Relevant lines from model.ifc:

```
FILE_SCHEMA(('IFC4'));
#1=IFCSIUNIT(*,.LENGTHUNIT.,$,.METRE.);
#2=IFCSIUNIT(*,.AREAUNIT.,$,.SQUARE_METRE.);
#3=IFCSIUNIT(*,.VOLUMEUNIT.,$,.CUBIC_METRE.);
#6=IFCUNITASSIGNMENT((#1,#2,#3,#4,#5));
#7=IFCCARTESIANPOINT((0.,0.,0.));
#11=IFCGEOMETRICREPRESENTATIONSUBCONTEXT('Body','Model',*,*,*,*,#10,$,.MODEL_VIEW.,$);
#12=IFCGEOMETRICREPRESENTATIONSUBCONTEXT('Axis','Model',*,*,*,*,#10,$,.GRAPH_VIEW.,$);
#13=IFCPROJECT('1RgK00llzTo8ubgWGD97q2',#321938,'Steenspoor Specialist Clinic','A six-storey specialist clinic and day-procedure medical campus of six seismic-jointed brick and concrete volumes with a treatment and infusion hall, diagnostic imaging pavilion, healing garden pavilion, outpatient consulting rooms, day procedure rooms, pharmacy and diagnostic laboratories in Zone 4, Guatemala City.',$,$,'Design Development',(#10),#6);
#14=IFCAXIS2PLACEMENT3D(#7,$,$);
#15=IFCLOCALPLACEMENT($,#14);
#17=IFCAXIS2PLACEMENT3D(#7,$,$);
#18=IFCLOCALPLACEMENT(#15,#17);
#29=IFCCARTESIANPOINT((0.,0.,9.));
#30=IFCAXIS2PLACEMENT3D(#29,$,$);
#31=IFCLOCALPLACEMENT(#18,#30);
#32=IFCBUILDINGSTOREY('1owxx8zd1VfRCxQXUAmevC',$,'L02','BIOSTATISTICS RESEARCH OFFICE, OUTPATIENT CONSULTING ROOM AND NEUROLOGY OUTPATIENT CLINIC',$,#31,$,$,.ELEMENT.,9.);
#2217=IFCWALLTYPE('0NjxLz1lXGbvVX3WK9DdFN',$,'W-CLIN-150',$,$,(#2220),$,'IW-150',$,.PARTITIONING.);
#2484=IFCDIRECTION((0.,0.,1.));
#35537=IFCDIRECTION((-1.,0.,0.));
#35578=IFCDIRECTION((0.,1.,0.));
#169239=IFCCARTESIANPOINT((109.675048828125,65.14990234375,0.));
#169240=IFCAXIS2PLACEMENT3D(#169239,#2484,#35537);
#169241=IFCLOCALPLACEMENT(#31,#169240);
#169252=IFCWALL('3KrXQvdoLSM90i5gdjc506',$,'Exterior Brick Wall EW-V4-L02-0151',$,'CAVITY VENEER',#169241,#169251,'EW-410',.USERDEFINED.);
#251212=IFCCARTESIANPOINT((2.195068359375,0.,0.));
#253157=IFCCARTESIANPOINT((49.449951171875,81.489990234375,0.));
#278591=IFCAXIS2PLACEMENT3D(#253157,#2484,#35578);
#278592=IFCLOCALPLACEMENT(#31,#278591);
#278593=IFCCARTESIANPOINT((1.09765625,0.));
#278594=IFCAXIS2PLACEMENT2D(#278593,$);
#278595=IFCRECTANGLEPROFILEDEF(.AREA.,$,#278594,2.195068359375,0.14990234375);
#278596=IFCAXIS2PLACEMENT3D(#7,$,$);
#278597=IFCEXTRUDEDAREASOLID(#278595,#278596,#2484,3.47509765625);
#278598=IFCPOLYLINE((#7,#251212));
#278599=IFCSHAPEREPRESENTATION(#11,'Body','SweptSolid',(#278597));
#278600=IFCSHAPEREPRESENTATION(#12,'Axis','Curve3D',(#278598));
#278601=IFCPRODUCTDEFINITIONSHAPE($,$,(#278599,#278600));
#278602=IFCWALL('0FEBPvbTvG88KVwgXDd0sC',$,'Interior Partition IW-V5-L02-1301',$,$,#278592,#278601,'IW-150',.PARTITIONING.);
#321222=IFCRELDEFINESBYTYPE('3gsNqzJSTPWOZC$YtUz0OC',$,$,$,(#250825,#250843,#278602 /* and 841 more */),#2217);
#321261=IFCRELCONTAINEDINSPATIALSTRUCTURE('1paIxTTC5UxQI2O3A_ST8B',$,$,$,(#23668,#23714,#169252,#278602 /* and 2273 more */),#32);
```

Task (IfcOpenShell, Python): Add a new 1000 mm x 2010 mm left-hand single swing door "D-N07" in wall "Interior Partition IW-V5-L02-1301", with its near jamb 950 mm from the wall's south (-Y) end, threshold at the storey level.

```python
import numpy as np
import ifcopenshell
import ifcopenshell.api.feature
import ifcopenshell.api.geometry
import ifcopenshell.api.root
import ifcopenshell.api.spatial
import ifcopenshell.geom
import ifcopenshell.util.element
import ifcopenshell.util.placement
import ifcopenshell.util.representation
import ifcopenshell.util.shape
import ifcopenshell.util.unit

model = ifcopenshell.open("model.ifc")
unit_scale = ifcopenshell.util.unit.calculate_unit_scale(model)
settings = ifcopenshell.geom.settings()


def volume(element):
    """Net volume in cubic metres, openings subtracted."""
    shape = ifcopenshell.geom.create_shape(settings, element)
    return ifcopenshell.util.shape.get_volume(shape.geometry)


wall = model.by_id(278602)
storey = ifcopenshell.util.element.get_container(wall, ifc_class="IfcBuildingStorey")
context = ifcopenshell.util.representation.get_context(model, "Model", "Body", "MODEL_VIEW")
before = volume(wall)

width, height, from_end, sill = 1, 2.01, 0.95, 0.0  # metres

# The wall runs along its own X axis, and the end named is its -X end.
wall_shape = ifcopenshell.geom.create_shape(settings, wall)
x, y, z = ifcopenshell.util.shape.get_vertices(wall_shape.geometry).T
start = x.min() + from_end
face, thickness = float(y.min()), float(y.max() - y.min())
wall_matrix = ifcopenshell.util.placement.get_local_placement(wall.ObjectPlacement)
level = ifcopenshell.util.placement.get_local_placement(storey.ObjectPlacement)[2, 3]


def in_wall(x, y):
    """Placement at x, y metres in the wall's axes, at sill height."""
    matrix = wall_matrix.copy()
    matrix[:, 3] = wall_matrix @ np.array([x / unit_scale, y / unit_scale, 0.0, 1.0])
    matrix[2, 3] = level + sill / unit_scale
    return matrix


# Opening: a box that overshoots both wall faces by 50 mm.
opening = ifcopenshell.api.root.create_entity(model, ifc_class="IfcOpeningElement", predefined_type="OPENING")
box = ifcopenshell.api.geometry.add_wall_representation(
    model, context=context, length=width, height=height, thickness=thickness + 0.1
)
ifcopenshell.api.geometry.assign_representation(model, product=opening, representation=box)
ifcopenshell.api.geometry.edit_object_placement(model, product=opening, matrix=in_wall(start, face - 0.05), is_si=False)
ifcopenshell.api.feature.add_feature(model, feature=opening, element=wall)

door = ifcopenshell.api.root.create_entity(model, ifc_class="IfcDoor", name="D-N07", predefined_type="DOOR")
door.OverallWidth, door.OverallHeight = width / unit_scale, height / unit_scale
door.OperationType = "SINGLE_SWING_LEFT"
body = ifcopenshell.api.geometry.add_door_representation(
    model,
    context=context,
    overall_width=door.OverallWidth,
    overall_height=door.OverallHeight,
    operation_type="SINGLE_SWING_LEFT",
    lining_properties={"LiningDepth": thickness / unit_scale, "ThresholdDepth": thickness / unit_scale},
)
ifcopenshell.api.geometry.assign_representation(model, product=door, representation=body)
ifcopenshell.api.spatial.assign_container(model, products=[door], relating_structure=storey)
ifcopenshell.api.feature.add_filling(model, opening=opening, element=door)

# The lining spans the wall, so the door starts at the wall face.
ifcopenshell.api.geometry.edit_object_placement(model, product=door, matrix=in_wall(start, face), is_si=False)

after = volume(wall)

print(f"wall volume {before:.3f} -> {after:.3f} m3")

model.write("model_edited.ifc")
```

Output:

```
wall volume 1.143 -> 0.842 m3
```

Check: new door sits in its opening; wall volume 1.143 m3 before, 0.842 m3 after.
